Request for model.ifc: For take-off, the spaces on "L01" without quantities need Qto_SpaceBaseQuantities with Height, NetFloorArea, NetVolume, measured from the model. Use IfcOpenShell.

First a look at what the model holds.

```python
import ifcopenshell
import ifcopenshell.util.element
import ifcopenshell.util.unit

model = ifcopenshell.open("model.ifc")
print(model.schema)
for unit_type in ("LENGTHUNIT", "AREAUNIT", "VOLUMEUNIT"):
    print(unit_type, ifcopenshell.util.unit.calculate_unit_scale(model, unit_type))
storey = next(s for s in model.by_type("IfcBuildingStorey") if s.Name == "L01")
spaces = [e for e in ifcopenshell.util.element.get_decomposition(storey) if e.is_a("IfcSpace")]
for e in sorted(spaces, key=lambda e: e.id()):
    print(e.id(), e.is_a(), e.Name, list(ifcopenshell.util.element.get_psets(e, qtos_only=True)), sep=" | ")
```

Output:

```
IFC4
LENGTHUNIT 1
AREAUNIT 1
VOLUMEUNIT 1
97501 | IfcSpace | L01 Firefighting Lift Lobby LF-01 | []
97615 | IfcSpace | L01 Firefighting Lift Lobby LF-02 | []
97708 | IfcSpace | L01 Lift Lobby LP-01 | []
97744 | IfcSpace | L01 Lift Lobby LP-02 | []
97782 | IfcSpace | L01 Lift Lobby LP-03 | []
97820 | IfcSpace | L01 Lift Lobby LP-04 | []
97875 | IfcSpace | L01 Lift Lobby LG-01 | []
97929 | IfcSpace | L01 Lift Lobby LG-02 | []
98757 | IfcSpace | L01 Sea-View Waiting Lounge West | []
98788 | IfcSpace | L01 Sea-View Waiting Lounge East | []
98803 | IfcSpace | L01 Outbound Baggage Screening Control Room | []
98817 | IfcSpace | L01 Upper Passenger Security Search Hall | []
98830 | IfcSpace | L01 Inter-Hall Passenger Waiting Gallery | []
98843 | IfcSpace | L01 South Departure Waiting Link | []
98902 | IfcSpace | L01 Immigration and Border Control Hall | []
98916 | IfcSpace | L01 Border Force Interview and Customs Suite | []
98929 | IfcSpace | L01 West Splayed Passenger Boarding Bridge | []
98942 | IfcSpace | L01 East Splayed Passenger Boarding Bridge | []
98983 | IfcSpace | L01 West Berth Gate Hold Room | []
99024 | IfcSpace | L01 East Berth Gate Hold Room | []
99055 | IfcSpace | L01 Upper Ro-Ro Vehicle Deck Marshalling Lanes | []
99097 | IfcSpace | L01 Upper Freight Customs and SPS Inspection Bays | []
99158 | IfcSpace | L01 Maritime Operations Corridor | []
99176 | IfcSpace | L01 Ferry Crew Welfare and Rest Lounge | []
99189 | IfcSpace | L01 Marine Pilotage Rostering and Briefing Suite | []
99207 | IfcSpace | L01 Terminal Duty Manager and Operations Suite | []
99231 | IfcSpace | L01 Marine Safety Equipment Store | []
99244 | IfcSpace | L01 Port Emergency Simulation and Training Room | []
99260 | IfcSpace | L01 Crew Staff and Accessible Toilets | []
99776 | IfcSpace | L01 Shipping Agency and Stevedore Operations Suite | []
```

```python
import ifcopenshell
import ifcopenshell.api.pset
import ifcopenshell.geom
import ifcopenshell.util.element
import ifcopenshell.util.shape
import ifcopenshell.util.unit

model = ifcopenshell.open("model.ifc")
unit_scale = ifcopenshell.util.unit.calculate_unit_scale(model)
area_scale = ifcopenshell.util.unit.calculate_unit_scale(model, "AREAUNIT")
volume_scale = ifcopenshell.util.unit.calculate_unit_scale(model, "VOLUMEUNIT")
settings = ifcopenshell.geom.settings()

storey = next(s for s in model.by_type("IfcBuildingStorey") if s.Name == "L01")
spaces = [e for e in ifcopenshell.util.element.get_decomposition(storey) if e.is_a("IfcSpace")]

for e in sorted(spaces, key=lambda e: e.id()):
    if ifcopenshell.util.element.get_psets(e, qtos_only=True, should_inherit=False):
        continue
    # Geometry comes back in metres, in the element's own axes.
    shape = ifcopenshell.geom.create_shape(settings, e)
    values = {
        "Height": ifcopenshell.util.shape.get_z(shape.geometry) / unit_scale,
        "NetFloorArea": ifcopenshell.util.shape.get_footprint_area(shape.geometry) / area_scale,
        "NetVolume": ifcopenshell.util.shape.get_volume(shape.geometry) / volume_scale,
    }
    qto = ifcopenshell.api.pset.add_qto(model, product=e, name="Qto_SpaceBaseQuantities")
    ifcopenshell.api.pset.edit_qto(model, qto=qto, properties=values)
    print(e.id(), {k: round(v, 3) for k, v in values.items()})

model.write("model-out.ifc")
```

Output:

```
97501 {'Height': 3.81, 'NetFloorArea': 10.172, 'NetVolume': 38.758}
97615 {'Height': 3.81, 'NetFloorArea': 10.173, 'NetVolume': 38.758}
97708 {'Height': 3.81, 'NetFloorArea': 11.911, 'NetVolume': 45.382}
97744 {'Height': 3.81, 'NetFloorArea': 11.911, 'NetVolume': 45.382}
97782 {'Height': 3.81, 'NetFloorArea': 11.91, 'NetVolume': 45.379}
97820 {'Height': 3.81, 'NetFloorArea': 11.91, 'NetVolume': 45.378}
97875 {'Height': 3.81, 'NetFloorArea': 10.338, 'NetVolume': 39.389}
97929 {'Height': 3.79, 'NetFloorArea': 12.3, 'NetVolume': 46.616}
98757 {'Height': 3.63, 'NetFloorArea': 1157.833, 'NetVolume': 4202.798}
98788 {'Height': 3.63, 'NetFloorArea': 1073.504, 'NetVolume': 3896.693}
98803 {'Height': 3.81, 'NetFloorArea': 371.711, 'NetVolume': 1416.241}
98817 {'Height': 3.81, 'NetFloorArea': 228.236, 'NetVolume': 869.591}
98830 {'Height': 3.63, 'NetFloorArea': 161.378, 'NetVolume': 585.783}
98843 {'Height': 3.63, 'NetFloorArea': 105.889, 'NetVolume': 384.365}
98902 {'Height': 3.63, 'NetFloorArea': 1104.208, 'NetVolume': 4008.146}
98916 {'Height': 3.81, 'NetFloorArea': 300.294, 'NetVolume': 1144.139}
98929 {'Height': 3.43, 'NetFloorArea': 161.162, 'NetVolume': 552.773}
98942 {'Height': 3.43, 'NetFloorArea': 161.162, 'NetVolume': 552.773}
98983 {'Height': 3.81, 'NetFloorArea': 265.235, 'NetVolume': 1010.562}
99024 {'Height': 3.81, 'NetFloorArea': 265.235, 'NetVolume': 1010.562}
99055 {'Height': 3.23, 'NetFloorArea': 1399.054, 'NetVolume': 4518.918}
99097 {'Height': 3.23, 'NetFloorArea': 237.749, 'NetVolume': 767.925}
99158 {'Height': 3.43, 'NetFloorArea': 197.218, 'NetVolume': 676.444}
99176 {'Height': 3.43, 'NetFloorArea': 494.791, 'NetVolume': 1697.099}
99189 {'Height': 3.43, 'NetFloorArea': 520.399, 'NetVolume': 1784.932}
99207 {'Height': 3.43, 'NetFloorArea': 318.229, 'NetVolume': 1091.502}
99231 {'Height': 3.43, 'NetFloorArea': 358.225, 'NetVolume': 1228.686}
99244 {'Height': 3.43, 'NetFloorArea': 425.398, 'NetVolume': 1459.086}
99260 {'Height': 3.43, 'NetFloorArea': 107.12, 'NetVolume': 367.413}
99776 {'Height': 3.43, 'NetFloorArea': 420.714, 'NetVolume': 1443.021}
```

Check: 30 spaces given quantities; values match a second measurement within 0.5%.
